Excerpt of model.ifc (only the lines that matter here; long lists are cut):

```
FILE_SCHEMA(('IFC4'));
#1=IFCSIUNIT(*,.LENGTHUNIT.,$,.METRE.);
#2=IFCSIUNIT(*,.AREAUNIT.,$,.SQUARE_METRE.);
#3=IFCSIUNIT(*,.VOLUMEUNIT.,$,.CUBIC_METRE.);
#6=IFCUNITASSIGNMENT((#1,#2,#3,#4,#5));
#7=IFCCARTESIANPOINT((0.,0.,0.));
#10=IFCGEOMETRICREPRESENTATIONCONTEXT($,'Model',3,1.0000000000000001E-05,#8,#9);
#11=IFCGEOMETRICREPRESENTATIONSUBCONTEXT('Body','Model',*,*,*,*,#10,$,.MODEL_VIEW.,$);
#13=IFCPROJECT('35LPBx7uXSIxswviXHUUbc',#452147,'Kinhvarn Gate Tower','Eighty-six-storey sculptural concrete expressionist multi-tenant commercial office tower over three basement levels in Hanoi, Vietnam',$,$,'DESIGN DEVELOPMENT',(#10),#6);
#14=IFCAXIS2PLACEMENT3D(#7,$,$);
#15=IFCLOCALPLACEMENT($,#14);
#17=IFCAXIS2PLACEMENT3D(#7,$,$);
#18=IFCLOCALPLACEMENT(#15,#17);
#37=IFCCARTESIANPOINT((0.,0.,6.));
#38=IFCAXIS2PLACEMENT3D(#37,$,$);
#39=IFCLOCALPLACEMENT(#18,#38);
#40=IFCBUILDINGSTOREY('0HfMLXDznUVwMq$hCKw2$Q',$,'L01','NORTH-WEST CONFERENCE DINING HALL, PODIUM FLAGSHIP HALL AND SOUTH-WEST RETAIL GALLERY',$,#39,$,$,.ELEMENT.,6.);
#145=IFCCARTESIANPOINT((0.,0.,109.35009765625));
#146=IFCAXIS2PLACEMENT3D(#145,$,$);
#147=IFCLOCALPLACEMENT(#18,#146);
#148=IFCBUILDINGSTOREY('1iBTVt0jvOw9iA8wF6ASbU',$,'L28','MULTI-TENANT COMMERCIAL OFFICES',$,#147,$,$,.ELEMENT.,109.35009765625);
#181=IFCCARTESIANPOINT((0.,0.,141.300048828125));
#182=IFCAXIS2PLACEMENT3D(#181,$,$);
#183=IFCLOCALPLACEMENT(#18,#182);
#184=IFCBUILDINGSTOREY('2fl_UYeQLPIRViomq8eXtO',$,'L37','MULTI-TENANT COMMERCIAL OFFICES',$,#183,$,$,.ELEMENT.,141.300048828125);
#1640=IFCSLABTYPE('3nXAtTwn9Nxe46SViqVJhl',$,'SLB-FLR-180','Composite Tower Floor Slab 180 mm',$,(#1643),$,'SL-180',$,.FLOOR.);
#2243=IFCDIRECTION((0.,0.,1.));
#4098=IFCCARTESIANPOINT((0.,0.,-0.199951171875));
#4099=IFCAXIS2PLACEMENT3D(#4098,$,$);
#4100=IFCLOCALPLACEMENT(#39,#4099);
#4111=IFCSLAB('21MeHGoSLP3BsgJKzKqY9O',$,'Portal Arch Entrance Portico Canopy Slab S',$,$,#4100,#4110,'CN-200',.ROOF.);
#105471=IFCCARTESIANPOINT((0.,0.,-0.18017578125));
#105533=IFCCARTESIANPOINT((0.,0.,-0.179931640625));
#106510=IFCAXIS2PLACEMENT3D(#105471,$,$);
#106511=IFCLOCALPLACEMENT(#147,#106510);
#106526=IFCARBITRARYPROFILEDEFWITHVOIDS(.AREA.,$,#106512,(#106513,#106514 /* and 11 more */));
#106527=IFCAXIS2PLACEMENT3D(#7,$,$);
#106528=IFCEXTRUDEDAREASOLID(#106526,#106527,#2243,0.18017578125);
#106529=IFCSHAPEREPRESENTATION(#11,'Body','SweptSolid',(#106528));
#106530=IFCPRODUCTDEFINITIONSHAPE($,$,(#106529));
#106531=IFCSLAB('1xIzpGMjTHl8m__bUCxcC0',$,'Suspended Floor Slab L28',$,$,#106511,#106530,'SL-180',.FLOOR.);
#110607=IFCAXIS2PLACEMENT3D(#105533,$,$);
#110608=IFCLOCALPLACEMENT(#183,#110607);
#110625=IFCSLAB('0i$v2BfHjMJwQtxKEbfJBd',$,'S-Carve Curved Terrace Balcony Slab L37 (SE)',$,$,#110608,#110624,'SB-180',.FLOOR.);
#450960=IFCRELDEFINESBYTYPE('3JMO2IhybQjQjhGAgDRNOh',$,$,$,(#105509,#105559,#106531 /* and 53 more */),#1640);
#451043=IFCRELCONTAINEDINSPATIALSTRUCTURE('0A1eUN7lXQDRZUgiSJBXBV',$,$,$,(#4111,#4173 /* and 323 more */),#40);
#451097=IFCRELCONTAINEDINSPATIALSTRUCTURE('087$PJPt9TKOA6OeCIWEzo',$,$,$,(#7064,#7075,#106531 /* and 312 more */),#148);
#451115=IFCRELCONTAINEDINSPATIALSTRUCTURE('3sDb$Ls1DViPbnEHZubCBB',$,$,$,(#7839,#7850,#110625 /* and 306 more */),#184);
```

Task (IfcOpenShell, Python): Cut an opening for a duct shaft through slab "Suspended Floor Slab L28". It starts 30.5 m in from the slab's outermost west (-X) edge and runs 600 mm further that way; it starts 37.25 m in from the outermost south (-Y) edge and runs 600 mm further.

```python
import numpy as np
import ifcopenshell
import ifcopenshell.api.feature
import ifcopenshell.api.geometry
import ifcopenshell.api.root
import ifcopenshell.geom
import ifcopenshell.util.placement
import ifcopenshell.util.representation
import ifcopenshell.util.shape
import ifcopenshell.util.unit

model = ifcopenshell.open("model.ifc")
unit_scale = ifcopenshell.util.unit.calculate_unit_scale(model)
settings = ifcopenshell.geom.settings()


def volume(element):
    """Net volume in cubic metres, openings subtracted."""
    shape = ifcopenshell.geom.create_shape(settings, element)
    return ifcopenshell.util.shape.get_volume(shape.geometry)


slab = model.by_guid("1xIzpGMjTHl8m__bUCxcC0")
before = volume(slab)

# Extent in the slab's own axes, in metres. The edges named are its -X and -Y sides.
slab_shape = ifcopenshell.geom.create_shape(settings, slab)
vertices = ifcopenshell.util.shape.get_vertices(slab_shape.geometry)
x_min, y_min, bottom = vertices.min(axis=0)
top = vertices[:, 2].max()

opening = ifcopenshell.api.root.create_entity(model, ifc_class="IfcOpeningElement", name="Duct shaft opening", predefined_type="OPENING")
context = ifcopenshell.util.representation.get_context(model, "Model", "Body", "MODEL_VIEW")
width, depth = 0.6, 0.6
outline = [(0.0, 0.0), (width, 0.0), (width, depth), (0.0, depth), (0.0, 0.0)]
# Overshoot both faces by 50 mm so the cut is clean.
shape = ifcopenshell.api.geometry.add_slab_representation(
    model, context=context, depth=top - bottom + 0.1, polyline=outline
)
ifcopenshell.api.geometry.assign_representation(model, product=opening, representation=shape)

matrix = ifcopenshell.util.placement.get_local_placement(slab.ObjectPlacement)
matrix[:, 3] = matrix @ np.append(np.array([x_min + 30.5, y_min + 37.25, bottom - 0.05]) / unit_scale, 1.0)
ifcopenshell.api.geometry.edit_object_placement(model, product=opening, matrix=matrix, is_si=False)
ifcopenshell.api.feature.add_feature(model, feature=opening, element=slab)

after = volume(slab)

print(f"slab volume {before:.3f} -> {after:.3f} m3")

model.write("model_rev.ifc")
```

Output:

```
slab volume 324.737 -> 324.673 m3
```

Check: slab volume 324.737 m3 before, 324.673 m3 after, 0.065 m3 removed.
